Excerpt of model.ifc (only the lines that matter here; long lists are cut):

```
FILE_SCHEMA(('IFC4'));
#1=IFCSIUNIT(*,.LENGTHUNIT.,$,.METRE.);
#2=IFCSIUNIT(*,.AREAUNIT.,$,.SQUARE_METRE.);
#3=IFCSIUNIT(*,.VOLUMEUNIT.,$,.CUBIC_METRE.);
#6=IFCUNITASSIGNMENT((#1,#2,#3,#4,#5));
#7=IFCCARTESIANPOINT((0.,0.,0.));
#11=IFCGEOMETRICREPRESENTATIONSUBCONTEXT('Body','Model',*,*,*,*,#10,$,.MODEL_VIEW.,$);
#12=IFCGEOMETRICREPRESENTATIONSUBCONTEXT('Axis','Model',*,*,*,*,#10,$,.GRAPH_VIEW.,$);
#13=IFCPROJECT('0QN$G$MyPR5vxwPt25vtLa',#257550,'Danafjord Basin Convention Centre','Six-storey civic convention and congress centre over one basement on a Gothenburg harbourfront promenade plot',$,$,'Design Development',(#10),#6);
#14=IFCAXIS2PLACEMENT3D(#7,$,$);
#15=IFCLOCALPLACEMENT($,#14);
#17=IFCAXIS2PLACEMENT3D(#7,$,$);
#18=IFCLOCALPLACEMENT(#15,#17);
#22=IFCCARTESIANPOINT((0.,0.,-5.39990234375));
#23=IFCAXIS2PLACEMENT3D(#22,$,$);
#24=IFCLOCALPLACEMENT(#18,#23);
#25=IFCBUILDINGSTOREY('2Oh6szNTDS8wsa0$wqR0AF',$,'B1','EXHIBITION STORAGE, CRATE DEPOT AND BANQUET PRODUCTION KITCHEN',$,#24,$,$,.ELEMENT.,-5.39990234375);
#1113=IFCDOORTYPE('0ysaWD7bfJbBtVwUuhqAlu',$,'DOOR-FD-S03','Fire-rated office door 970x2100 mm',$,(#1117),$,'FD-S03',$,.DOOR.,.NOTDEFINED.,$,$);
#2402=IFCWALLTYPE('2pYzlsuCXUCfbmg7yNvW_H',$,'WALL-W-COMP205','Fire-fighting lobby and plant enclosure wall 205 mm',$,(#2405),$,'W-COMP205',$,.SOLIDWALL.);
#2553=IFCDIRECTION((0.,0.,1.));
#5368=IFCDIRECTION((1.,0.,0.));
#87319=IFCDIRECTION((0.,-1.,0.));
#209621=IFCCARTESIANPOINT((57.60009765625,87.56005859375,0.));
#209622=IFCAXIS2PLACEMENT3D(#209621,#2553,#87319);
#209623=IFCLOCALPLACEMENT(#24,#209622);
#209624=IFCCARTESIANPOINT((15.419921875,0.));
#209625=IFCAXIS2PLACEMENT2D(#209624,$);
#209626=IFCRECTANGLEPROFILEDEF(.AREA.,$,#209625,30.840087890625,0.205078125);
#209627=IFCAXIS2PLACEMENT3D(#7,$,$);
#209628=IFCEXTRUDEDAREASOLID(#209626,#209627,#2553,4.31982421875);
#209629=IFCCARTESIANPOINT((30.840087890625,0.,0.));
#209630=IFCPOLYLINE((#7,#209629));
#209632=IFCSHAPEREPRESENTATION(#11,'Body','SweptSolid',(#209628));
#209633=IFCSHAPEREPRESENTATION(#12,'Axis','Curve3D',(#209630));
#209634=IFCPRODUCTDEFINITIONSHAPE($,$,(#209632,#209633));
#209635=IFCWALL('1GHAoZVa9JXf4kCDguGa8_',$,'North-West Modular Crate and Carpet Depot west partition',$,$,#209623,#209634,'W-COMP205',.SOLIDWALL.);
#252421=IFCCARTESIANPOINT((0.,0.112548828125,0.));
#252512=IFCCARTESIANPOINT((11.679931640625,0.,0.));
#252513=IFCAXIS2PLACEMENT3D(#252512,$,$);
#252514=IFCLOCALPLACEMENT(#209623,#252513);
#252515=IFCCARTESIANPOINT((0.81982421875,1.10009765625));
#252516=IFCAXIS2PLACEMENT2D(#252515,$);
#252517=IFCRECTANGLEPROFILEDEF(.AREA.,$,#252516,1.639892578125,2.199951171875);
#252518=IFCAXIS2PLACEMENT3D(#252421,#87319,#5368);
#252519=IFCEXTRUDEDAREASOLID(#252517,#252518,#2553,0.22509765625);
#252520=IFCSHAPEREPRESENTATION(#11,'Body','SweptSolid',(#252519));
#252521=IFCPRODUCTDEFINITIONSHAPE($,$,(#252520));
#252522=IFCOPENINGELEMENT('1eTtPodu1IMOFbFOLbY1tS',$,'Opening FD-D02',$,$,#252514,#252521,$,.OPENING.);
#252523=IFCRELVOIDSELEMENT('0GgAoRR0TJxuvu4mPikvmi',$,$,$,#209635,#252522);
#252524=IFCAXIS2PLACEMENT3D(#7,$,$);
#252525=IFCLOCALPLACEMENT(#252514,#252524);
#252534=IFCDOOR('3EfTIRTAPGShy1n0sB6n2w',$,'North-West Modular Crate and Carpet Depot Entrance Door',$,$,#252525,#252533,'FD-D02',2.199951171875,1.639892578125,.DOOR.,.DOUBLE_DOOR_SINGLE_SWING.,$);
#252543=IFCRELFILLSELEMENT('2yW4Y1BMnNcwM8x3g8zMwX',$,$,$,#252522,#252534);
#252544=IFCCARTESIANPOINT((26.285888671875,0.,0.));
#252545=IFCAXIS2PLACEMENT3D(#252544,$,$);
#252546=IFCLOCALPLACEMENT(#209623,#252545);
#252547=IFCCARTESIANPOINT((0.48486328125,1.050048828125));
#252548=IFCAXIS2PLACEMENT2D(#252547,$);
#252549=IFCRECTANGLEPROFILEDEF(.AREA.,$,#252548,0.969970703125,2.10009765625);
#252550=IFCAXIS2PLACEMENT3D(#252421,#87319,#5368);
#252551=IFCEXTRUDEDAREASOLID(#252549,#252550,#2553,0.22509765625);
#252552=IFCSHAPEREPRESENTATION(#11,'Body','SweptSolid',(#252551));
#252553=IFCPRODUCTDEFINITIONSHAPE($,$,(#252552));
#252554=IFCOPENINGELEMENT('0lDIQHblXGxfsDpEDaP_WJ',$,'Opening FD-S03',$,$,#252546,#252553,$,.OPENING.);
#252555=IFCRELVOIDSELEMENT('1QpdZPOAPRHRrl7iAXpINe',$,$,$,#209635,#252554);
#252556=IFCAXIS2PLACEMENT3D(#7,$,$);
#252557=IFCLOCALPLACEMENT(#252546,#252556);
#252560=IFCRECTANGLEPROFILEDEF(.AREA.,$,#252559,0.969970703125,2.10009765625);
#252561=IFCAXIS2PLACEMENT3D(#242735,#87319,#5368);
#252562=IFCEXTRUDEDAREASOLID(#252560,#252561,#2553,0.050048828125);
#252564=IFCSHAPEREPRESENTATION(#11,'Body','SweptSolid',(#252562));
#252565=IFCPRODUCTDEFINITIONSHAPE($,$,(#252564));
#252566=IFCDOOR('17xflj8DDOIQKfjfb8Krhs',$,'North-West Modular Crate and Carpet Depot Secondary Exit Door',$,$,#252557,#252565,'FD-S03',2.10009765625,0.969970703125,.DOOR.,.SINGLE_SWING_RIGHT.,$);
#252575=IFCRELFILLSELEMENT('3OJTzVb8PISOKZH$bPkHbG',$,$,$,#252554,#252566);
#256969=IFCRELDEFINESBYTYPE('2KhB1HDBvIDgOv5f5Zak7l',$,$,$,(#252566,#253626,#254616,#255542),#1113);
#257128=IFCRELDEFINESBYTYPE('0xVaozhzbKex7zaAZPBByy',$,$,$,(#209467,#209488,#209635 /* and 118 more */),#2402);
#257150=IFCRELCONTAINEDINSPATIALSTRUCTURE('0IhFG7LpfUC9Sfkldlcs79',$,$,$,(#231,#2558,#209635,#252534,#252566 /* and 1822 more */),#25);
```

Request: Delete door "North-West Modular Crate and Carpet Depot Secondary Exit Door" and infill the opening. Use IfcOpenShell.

```python
import ifcopenshell
import ifcopenshell.api.feature
import ifcopenshell.api.root
import ifcopenshell.geom
import ifcopenshell.util.shape

model = ifcopenshell.open("model.ifc")
settings = ifcopenshell.geom.settings()


def volume(element):
    """Net volume in cubic metres, openings subtracted."""
    shape = ifcopenshell.geom.create_shape(settings, element)
    return ifcopenshell.util.shape.get_volume(shape.geometry)


door = model.by_guid("17xflj8DDOIQKfjfb8Krhs")
opening = door.FillsVoids[0].RelatingOpeningElement
wall = opening.VoidsElements[0].RelatingBuildingElement
before = volume(wall)

ifcopenshell.api.root.remove_product(model, product=door)
ifcopenshell.api.feature.remove_feature(model, feature=opening)

after = volume(wall)

print(f"wall volume {before:.3f} -> {after:.3f} m3")

model.write("model_edited.ifc")
```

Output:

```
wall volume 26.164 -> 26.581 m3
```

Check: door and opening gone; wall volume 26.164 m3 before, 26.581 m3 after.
